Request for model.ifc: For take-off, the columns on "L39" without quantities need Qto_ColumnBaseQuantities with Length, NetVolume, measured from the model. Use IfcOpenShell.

First a look at what the model holds.

```python
import ifcopenshell
import ifcopenshell.util.element
import ifcopenshell.util.unit

model = ifcopenshell.open("model.ifc")
print(model.schema)
for unit_type in ("LENGTHUNIT", "AREAUNIT", "VOLUMEUNIT"):
    print(unit_type, ifcopenshell.util.unit.calculate_unit_scale(model, unit_type))
storey = next(s for s in model.by_type("IfcBuildingStorey") if s.Name == "L39")
columns = [e for e in ifcopenshell.util.element.get_decomposition(storey) if e.is_a("IfcColumn")]
for e in sorted(columns, key=lambda e: e.id()):
    print(e.id(), e.is_a(), e.Name, list(ifcopenshell.util.element.get_psets(e, qtos_only=True)), sep=" | ")
```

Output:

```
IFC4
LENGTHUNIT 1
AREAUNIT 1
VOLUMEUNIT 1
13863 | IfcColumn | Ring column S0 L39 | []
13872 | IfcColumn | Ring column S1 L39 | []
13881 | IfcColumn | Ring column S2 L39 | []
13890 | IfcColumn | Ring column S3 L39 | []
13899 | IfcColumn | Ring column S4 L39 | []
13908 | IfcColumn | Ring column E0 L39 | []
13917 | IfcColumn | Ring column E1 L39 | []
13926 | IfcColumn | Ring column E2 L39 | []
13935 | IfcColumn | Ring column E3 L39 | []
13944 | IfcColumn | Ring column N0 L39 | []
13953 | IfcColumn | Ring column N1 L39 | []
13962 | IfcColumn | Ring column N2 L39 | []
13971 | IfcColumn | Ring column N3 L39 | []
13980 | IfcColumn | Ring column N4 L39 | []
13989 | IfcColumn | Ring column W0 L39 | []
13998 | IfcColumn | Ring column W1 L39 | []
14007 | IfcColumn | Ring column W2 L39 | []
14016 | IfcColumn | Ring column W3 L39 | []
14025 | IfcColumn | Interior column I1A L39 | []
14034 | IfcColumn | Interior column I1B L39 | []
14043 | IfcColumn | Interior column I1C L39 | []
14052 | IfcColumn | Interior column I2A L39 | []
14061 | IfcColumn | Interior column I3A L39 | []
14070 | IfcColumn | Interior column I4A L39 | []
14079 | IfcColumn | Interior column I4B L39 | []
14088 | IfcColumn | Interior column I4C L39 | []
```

```python
import ifcopenshell
import ifcopenshell.api.pset
import ifcopenshell.geom
import ifcopenshell.util.element
import ifcopenshell.util.shape
import ifcopenshell.util.unit

model = ifcopenshell.open("model.ifc")
unit_scale = ifcopenshell.util.unit.calculate_unit_scale(model)
volume_scale = ifcopenshell.util.unit.calculate_unit_scale(model, "VOLUMEUNIT")
settings = ifcopenshell.geom.settings()

storey = next(s for s in model.by_type("IfcBuildingStorey") if s.Name == "L39")
columns = [e for e in ifcopenshell.util.element.get_decomposition(storey) if e.is_a("IfcColumn")]

for e in sorted(columns, key=lambda e: e.id()):
    if ifcopenshell.util.element.get_psets(e, qtos_only=True, should_inherit=False):
        continue
    # Geometry comes back in metres, in the element's own axes.
    shape = ifcopenshell.geom.create_shape(settings, e)
    values = {
        "Length": ifcopenshell.util.shape.get_z(shape.geometry) / unit_scale,
        "NetVolume": ifcopenshell.util.shape.get_volume(shape.geometry) / volume_scale,
    }
    qto = ifcopenshell.api.pset.add_qto(model, product=e, name="Qto_ColumnBaseQuantities")
    ifcopenshell.api.pset.edit_qto(model, qto=qto, properties=values)
    print(e.id(), {k: round(v, 3) for k, v in values.items()})

model.write("model_v2.ifc")
```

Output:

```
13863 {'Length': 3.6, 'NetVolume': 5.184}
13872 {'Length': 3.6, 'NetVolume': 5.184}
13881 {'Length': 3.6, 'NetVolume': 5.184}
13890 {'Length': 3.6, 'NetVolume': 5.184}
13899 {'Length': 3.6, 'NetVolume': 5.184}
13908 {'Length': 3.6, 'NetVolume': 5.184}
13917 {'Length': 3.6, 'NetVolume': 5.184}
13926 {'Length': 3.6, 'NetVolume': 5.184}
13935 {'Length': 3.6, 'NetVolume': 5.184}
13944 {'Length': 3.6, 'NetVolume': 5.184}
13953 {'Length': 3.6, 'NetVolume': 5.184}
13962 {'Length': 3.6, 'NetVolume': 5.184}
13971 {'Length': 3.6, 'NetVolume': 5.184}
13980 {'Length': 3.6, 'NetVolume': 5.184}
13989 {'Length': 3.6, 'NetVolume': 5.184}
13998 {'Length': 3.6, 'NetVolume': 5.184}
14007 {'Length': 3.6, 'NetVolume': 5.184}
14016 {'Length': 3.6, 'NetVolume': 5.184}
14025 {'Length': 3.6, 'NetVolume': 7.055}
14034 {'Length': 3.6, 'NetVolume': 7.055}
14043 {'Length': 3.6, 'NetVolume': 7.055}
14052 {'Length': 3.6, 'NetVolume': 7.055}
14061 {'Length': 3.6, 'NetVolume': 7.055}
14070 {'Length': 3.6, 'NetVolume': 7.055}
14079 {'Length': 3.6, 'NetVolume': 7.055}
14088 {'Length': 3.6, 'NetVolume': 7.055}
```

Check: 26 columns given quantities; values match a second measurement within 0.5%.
